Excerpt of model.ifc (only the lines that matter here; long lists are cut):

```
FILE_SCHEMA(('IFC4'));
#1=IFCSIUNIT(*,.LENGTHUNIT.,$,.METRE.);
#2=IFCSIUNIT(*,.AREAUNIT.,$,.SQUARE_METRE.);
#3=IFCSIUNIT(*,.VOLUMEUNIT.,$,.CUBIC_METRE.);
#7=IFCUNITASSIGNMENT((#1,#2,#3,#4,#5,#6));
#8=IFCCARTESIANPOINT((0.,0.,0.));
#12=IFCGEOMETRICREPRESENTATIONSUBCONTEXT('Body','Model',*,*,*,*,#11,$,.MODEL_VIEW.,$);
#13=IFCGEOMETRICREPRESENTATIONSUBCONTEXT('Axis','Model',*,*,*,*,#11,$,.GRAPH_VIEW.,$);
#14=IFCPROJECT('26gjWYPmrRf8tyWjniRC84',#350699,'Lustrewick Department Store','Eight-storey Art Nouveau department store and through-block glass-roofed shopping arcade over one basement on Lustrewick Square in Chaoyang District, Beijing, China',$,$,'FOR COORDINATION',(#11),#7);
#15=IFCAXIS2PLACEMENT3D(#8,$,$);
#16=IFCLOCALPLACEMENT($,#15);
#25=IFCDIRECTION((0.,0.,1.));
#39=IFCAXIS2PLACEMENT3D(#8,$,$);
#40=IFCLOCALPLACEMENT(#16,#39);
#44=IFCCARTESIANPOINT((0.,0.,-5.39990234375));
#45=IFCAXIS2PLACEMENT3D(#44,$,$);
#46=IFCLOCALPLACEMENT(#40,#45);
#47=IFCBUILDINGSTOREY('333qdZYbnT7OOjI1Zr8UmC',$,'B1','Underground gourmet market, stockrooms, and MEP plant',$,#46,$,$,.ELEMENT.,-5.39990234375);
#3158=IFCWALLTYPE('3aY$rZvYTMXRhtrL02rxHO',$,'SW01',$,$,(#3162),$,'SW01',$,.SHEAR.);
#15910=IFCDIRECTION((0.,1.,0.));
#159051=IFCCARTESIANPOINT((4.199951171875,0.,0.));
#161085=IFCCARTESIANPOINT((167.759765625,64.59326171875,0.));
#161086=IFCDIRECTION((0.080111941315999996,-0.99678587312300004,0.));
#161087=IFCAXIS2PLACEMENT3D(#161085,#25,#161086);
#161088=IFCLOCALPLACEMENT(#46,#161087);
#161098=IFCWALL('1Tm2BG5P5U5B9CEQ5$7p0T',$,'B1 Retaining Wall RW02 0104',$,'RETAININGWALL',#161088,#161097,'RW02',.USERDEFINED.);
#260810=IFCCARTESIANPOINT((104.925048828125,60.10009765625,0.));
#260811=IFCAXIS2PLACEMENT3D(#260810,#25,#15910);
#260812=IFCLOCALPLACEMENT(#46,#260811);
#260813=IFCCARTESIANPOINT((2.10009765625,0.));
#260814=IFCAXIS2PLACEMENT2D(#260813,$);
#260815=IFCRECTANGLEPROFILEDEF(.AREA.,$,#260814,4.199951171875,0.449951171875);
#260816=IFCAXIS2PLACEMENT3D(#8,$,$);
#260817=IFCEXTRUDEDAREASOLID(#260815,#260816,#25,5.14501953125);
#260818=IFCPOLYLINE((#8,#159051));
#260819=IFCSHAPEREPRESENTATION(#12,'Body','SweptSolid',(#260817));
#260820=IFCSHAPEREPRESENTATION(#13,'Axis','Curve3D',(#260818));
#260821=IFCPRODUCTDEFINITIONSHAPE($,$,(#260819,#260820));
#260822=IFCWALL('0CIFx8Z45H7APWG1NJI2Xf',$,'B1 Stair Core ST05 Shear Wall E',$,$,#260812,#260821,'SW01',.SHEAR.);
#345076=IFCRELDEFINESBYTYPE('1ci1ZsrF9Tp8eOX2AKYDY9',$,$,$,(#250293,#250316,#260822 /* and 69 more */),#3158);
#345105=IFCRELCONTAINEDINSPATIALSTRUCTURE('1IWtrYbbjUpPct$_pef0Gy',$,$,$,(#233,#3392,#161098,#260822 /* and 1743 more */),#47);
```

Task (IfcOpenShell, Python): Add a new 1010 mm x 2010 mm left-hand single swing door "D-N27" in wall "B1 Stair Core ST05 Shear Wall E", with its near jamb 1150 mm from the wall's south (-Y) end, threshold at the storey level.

```python
import numpy as np
import ifcopenshell
import ifcopenshell.api.feature
import ifcopenshell.api.geometry
import ifcopenshell.api.root
import ifcopenshell.api.spatial
import ifcopenshell.geom
import ifcopenshell.util.element
import ifcopenshell.util.placement
import ifcopenshell.util.representation
import ifcopenshell.util.shape
import ifcopenshell.util.unit

model = ifcopenshell.open("model.ifc")
unit_scale = ifcopenshell.util.unit.calculate_unit_scale(model)
settings = ifcopenshell.geom.settings()


def volume(element):
    """Net volume in cubic metres, openings subtracted."""
    shape = ifcopenshell.geom.create_shape(settings, element)
    return ifcopenshell.util.shape.get_volume(shape.geometry)


wall = model.by_guid("0CIFx8Z45H7APWG1NJI2Xf")
storey = ifcopenshell.util.element.get_container(wall, ifc_class="IfcBuildingStorey")
context = ifcopenshell.util.representation.get_context(model, "Model", "Body", "MODEL_VIEW")
before = volume(wall)

width, height, from_end, sill = 1.01, 2.01, 1.15, 0.0  # metres

# The wall runs along its own X axis, and the end named is its -X end.
wall_shape = ifcopenshell.geom.create_shape(settings, wall)
x, y, z = ifcopenshell.util.shape.get_vertices(wall_shape.geometry).T
start = x.min() + from_end
face, thickness = float(y.min()), float(y.max() - y.min())
wall_matrix = ifcopenshell.util.placement.get_local_placement(wall.ObjectPlacement)
level = ifcopenshell.util.placement.get_local_placement(storey.ObjectPlacement)[2, 3]


def in_wall(x, y):
    """Placement at x, y metres in the wall's axes, at sill height."""
    matrix = wall_matrix.copy()
    matrix[:, 3] = wall_matrix @ np.array([x / unit_scale, y / unit_scale, 0.0, 1.0])
    matrix[2, 3] = level + sill / unit_scale
    return matrix


# Opening: a box that overshoots both wall faces by 50 mm.
opening = ifcopenshell.api.root.create_entity(model, ifc_class="IfcOpeningElement", predefined_type="OPENING")
box = ifcopenshell.api.geometry.add_wall_representation(
    model, context=context, length=width, height=height, thickness=thickness + 0.1
)
ifcopenshell.api.geometry.assign_representation(model, product=opening, representation=box)
ifcopenshell.api.geometry.edit_object_placement(model, product=opening, matrix=in_wall(start, face - 0.05), is_si=False)
ifcopenshell.api.feature.add_feature(model, feature=opening, element=wall)

door = ifcopenshell.api.root.create_entity(model, ifc_class="IfcDoor", name="D-N27", predefined_type="DOOR")
door.OverallWidth, door.OverallHeight = width / unit_scale, height / unit_scale
door.OperationType = "SINGLE_SWING_LEFT"
body = ifcopenshell.api.geometry.add_door_representation(
    model,
    context=context,
    overall_width=door.OverallWidth,
    overall_height=door.OverallHeight,
    operation_type="SINGLE_SWING_LEFT",
    lining_properties={"LiningDepth": thickness / unit_scale, "ThresholdDepth": thickness / unit_scale},
)
ifcopenshell.api.geometry.assign_representation(model, product=door, representation=body)
ifcopenshell.api.spatial.assign_container(model, products=[door], relating_structure=storey)
ifcopenshell.api.feature.add_filling(model, opening=opening, element=door)

# The lining spans the wall, so the door starts at the wall face.
ifcopenshell.api.geometry.edit_object_placement(model, product=door, matrix=in_wall(start, face), is_si=False)

after = volume(wall)

print(f"wall volume {before:.3f} -> {after:.3f} m3")

model.write("model_rev.ifc")
```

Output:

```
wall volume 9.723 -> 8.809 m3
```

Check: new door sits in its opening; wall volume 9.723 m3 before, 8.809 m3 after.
